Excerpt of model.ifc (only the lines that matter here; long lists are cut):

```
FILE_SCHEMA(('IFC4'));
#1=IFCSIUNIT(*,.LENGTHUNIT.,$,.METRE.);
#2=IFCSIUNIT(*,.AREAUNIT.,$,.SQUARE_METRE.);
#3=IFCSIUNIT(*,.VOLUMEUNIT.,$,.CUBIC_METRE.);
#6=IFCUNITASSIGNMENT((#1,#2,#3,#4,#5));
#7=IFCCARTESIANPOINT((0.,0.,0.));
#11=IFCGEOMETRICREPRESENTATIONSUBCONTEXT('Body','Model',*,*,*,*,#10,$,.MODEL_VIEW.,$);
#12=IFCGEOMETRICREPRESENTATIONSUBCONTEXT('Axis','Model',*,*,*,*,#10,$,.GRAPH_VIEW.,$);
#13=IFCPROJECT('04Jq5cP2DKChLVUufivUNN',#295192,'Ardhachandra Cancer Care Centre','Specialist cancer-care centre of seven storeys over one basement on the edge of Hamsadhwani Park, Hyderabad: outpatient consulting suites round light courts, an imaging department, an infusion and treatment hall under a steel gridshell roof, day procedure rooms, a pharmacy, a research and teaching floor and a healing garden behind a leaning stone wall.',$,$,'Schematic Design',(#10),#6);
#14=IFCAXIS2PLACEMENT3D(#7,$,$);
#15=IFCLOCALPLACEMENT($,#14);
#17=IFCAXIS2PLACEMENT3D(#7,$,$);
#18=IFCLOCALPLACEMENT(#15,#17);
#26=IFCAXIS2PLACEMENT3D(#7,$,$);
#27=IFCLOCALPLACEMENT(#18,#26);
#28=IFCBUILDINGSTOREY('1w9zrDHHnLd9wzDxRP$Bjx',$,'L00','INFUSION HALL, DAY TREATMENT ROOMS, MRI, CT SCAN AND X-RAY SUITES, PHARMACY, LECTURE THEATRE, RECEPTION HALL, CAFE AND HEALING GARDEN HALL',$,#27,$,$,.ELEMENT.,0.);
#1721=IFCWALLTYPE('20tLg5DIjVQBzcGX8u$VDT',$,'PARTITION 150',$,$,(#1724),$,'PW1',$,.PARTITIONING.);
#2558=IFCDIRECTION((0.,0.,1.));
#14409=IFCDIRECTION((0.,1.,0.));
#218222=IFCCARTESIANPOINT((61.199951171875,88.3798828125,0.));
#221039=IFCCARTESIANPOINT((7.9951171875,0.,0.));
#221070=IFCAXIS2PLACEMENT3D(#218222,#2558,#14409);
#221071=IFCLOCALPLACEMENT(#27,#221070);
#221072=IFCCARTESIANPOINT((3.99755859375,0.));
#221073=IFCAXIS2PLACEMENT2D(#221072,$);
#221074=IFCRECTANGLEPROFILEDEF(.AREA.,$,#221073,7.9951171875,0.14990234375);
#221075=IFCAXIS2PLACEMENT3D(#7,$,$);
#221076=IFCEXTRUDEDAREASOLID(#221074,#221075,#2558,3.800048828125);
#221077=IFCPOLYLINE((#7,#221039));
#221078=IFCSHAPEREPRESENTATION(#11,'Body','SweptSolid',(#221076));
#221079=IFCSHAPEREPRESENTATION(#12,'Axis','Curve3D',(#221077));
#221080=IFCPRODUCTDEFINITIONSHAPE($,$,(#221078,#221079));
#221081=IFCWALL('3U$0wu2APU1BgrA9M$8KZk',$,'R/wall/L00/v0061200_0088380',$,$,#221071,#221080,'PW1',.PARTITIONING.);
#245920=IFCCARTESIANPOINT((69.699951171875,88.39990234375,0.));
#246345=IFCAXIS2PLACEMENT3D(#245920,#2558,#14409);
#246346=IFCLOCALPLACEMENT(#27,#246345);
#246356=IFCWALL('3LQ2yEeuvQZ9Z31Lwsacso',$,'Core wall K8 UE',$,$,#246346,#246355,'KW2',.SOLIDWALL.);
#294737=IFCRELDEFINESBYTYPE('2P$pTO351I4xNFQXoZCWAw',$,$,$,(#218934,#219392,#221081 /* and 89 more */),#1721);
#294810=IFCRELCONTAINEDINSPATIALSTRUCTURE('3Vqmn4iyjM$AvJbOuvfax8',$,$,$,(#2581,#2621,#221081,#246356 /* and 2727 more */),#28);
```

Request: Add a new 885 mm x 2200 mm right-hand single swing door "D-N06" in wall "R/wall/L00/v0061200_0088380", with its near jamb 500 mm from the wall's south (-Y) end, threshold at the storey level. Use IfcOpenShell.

```python
import numpy as np
import ifcopenshell
import ifcopenshell.api.feature
import ifcopenshell.api.geometry
import ifcopenshell.api.root
import ifcopenshell.api.spatial
import ifcopenshell.geom
import ifcopenshell.util.element
import ifcopenshell.util.placement
import ifcopenshell.util.representation
import ifcopenshell.util.shape
import ifcopenshell.util.unit

model = ifcopenshell.open("model.ifc")
unit_scale = ifcopenshell.util.unit.calculate_unit_scale(model)
settings = ifcopenshell.geom.settings()


def volume(element):
    """Net volume in cubic metres, openings subtracted."""
    shape = ifcopenshell.geom.create_shape(settings, element)
    return ifcopenshell.util.shape.get_volume(shape.geometry)


wall = model.by_guid("3U$0wu2APU1BgrA9M$8KZk")
storey = ifcopenshell.util.element.get_container(wall, ifc_class="IfcBuildingStorey")
context = ifcopenshell.util.representation.get_context(model, "Model", "Body", "MODEL_VIEW")
before = volume(wall)

width, height, from_end, sill = 0.885, 2.2, 0.5, 0.0  # metres

# The wall runs along its own X axis, and the end named is its -X end.
wall_shape = ifcopenshell.geom.create_shape(settings, wall)
x, y, z = ifcopenshell.util.shape.get_vertices(wall_shape.geometry).T
start = x.min() + from_end
face, thickness = float(y.min()), float(y.max() - y.min())
wall_matrix = ifcopenshell.util.placement.get_local_placement(wall.ObjectPlacement)
level = ifcopenshell.util.placement.get_local_placement(storey.ObjectPlacement)[2, 3]


def in_wall(x, y):
    """Placement at x, y metres in the wall's axes, at sill height."""
    matrix = wall_matrix.copy()
    matrix[:, 3] = wall_matrix @ np.array([x / unit_scale, y / unit_scale, 0.0, 1.0])
    matrix[2, 3] = level + sill / unit_scale
    return matrix


# Opening: a box that overshoots both wall faces by 50 mm.
opening = ifcopenshell.api.root.create_entity(model, ifc_class="IfcOpeningElement", predefined_type="OPENING")
box = ifcopenshell.api.geometry.add_wall_representation(
    model, context=context, length=width, height=height, thickness=thickness + 0.1
)
ifcopenshell.api.geometry.assign_representation(model, product=opening, representation=box)
ifcopenshell.api.geometry.edit_object_placement(model, product=opening, matrix=in_wall(start, face - 0.05), is_si=False)
ifcopenshell.api.feature.add_feature(model, feature=opening, element=wall)

door = ifcopenshell.api.root.create_entity(model, ifc_class="IfcDoor", name="D-N06", predefined_type="DOOR")
door.OverallWidth, door.OverallHeight = width / unit_scale, height / unit_scale
door.OperationType = "SINGLE_SWING_RIGHT"
body = ifcopenshell.api.geometry.add_door_representation(
    model,
    context=context,
    overall_width=door.OverallWidth,
    overall_height=door.OverallHeight,
    operation_type="SINGLE_SWING_RIGHT",
    lining_properties={"LiningDepth": thickness / unit_scale, "ThresholdDepth": thickness / unit_scale},
)
ifcopenshell.api.geometry.assign_representation(model, product=door, representation=body)
ifcopenshell.api.spatial.assign_container(model, products=[door], relating_structure=storey)
ifcopenshell.api.feature.add_filling(model, opening=opening, element=door)

# The lining spans the wall, so the door starts at the wall face.
ifcopenshell.api.geometry.edit_object_placement(model, product=door, matrix=in_wall(start, face), is_si=False)

after = volume(wall)

print(f"wall volume {before:.3f} -> {after:.3f} m3")

model.write("model_v2.ifc")
```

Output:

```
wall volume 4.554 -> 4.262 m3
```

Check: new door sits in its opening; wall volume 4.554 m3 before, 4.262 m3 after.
